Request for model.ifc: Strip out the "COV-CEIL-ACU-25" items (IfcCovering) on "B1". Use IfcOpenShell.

First a look at what the model holds.

```python
import ifcopenshell
import ifcopenshell.util.element

model = ifcopenshell.open("model.ifc")
print(model.schema)
storey = next(s for s in model.by_type("IfcBuildingStorey") if s.Name == "B1")
coverings = [e for e in ifcopenshell.util.element.get_decomposition(storey) if e.is_a("IfcCovering")]
seen = {}
for e in coverings:
    element_type = ifcopenshell.util.element.get_type(e)
    name = element_type.Name if element_type not in (None, e) else None
    seen[name] = seen.get(name, 0) + 1
for name, count in sorted(seen.items(), key=str):
    print(count, "x", name)
```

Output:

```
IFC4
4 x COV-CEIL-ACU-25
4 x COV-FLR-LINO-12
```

```python
import ifcopenshell
import ifcopenshell.api.root
import ifcopenshell.util.element

model = ifcopenshell.open("model.ifc")

storey = next(s for s in model.by_type("IfcBuildingStorey") if s.Name == "B1")
coverings = [e for e in ifcopenshell.util.element.get_decomposition(storey) if e.is_a("IfcCovering")]
targets = [e for e in coverings if (t := ifcopenshell.util.element.get_type(e)) not in (None, e) and t.Name == "COV-CEIL-ACU-25"]

for e in targets:
    ifcopenshell.api.root.remove_product(model, product=e)
print(len(targets), "removed")

model.write("model-out.ifc")
```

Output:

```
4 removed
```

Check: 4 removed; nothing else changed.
